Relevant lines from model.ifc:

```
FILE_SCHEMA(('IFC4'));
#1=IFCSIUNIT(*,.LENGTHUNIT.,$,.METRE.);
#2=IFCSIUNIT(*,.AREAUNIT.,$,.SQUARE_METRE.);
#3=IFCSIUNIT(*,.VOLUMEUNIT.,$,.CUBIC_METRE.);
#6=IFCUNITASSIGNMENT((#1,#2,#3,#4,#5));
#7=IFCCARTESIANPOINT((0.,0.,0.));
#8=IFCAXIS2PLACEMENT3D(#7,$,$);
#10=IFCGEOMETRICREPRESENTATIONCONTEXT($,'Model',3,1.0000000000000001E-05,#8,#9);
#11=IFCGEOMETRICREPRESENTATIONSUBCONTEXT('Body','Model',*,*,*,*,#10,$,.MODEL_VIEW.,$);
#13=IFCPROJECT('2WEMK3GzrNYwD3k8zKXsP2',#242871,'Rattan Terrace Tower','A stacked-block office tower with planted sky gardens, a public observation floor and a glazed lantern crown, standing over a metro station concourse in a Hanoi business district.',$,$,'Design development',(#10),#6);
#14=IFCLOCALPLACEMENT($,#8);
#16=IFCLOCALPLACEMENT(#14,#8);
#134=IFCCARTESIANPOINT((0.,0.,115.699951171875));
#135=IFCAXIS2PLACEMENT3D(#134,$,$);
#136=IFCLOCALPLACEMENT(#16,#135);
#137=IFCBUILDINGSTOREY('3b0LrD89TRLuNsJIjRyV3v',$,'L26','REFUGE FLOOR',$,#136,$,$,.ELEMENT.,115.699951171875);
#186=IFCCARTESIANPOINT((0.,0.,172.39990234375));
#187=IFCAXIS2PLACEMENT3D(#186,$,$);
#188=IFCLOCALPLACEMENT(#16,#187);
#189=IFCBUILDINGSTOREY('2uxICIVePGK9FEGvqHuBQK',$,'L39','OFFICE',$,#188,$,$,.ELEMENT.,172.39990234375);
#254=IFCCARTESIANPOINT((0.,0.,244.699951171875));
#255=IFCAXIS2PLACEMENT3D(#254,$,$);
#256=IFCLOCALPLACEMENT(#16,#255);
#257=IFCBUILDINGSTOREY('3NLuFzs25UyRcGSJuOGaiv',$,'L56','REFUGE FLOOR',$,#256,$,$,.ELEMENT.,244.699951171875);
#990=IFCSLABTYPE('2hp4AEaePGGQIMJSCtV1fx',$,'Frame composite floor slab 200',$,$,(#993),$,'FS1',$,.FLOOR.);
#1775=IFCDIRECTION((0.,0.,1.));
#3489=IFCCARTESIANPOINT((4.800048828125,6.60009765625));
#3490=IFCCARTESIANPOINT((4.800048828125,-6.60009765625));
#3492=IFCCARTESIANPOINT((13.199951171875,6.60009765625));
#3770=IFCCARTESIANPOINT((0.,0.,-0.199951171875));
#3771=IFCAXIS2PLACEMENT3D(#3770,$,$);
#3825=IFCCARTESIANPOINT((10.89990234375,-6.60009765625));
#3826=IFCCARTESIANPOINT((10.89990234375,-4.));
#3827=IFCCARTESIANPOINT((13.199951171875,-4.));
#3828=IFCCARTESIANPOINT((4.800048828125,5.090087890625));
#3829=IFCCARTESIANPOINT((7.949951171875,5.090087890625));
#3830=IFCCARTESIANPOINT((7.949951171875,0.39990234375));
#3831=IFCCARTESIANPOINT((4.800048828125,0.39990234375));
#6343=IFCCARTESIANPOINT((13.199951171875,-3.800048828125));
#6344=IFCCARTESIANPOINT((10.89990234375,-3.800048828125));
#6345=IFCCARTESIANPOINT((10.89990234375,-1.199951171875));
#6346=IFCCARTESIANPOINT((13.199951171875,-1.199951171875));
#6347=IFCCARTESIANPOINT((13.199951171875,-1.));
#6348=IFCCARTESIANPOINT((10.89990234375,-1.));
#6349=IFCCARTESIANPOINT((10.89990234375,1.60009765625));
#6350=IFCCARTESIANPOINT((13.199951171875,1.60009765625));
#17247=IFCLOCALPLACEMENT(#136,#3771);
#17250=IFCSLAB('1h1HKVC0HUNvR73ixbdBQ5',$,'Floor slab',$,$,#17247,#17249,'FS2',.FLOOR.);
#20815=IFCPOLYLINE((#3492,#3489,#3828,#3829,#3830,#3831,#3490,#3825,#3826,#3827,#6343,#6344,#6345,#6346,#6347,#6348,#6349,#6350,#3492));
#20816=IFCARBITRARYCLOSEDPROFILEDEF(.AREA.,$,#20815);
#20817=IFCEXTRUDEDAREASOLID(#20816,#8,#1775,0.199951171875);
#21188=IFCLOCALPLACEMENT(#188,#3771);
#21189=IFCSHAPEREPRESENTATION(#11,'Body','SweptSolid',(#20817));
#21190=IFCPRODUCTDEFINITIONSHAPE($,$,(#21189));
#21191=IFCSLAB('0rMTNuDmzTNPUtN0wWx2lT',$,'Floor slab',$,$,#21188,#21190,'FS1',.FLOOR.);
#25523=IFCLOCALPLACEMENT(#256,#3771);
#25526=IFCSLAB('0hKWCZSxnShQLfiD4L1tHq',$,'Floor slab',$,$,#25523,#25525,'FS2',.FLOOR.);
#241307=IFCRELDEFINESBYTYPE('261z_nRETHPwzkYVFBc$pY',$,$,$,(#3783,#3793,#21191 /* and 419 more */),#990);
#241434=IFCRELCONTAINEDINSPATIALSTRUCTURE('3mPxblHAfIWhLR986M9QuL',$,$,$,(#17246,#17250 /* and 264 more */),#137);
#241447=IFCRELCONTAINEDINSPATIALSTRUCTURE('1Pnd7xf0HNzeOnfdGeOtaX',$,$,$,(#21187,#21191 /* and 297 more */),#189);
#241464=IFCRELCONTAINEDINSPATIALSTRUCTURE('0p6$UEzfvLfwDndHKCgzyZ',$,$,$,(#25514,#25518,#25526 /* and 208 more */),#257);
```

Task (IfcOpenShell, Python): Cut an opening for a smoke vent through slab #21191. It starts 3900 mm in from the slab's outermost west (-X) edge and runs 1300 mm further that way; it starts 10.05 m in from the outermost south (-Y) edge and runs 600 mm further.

```python
import numpy as np
import ifcopenshell
import ifcopenshell.api.feature
import ifcopenshell.api.geometry
import ifcopenshell.api.root
import ifcopenshell.geom
import ifcopenshell.util.placement
import ifcopenshell.util.representation
import ifcopenshell.util.shape
import ifcopenshell.util.unit

model = ifcopenshell.open("model.ifc")
unit_scale = ifcopenshell.util.unit.calculate_unit_scale(model)
settings = ifcopenshell.geom.settings()


def volume(element):
    """Net volume in cubic metres, openings subtracted."""
    shape = ifcopenshell.geom.create_shape(settings, element)
    return ifcopenshell.util.shape.get_volume(shape.geometry)


slab = model.by_guid("0rMTNuDmzTNPUtN0wWx2lT")
before = volume(slab)

# Extent in the slab's own axes, in metres. The edges named are its -X and -Y sides.
slab_shape = ifcopenshell.geom.create_shape(settings, slab)
vertices = ifcopenshell.util.shape.get_vertices(slab_shape.geometry)
x_min, y_min, bottom = vertices.min(axis=0)
top = vertices[:, 2].max()

opening = ifcopenshell.api.root.create_entity(model, ifc_class="IfcOpeningElement", name="Smoke vent opening", predefined_type="OPENING")
context = ifcopenshell.util.representation.get_context(model, "Model", "Body", "MODEL_VIEW")
width, depth = 1.3, 0.6
outline = [(0.0, 0.0), (width, 0.0), (width, depth), (0.0, depth), (0.0, 0.0)]
# Overshoot both faces by 50 mm so the cut is clean.
shape = ifcopenshell.api.geometry.add_slab_representation(
    model, context=context, depth=top - bottom + 0.1, polyline=outline
)
ifcopenshell.api.geometry.assign_representation(model, product=opening, representation=shape)

matrix = ifcopenshell.util.placement.get_local_placement(slab.ObjectPlacement)
matrix[:, 3] = matrix @ np.append(np.array([x_min + 3.9, y_min + 10.05, bottom - 0.05]) / unit_scale, 1.0)
ifcopenshell.api.geometry.edit_object_placement(model, product=opening, matrix=matrix, is_si=False)
ifcopenshell.api.feature.add_feature(model, feature=opening, element=slab)

after = volume(slab)

print(f"slab volume {before:.3f} -> {after:.3f} m3")

model.write("model_updated.ifc")
```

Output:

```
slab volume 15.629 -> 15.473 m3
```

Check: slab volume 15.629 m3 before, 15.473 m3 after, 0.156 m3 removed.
